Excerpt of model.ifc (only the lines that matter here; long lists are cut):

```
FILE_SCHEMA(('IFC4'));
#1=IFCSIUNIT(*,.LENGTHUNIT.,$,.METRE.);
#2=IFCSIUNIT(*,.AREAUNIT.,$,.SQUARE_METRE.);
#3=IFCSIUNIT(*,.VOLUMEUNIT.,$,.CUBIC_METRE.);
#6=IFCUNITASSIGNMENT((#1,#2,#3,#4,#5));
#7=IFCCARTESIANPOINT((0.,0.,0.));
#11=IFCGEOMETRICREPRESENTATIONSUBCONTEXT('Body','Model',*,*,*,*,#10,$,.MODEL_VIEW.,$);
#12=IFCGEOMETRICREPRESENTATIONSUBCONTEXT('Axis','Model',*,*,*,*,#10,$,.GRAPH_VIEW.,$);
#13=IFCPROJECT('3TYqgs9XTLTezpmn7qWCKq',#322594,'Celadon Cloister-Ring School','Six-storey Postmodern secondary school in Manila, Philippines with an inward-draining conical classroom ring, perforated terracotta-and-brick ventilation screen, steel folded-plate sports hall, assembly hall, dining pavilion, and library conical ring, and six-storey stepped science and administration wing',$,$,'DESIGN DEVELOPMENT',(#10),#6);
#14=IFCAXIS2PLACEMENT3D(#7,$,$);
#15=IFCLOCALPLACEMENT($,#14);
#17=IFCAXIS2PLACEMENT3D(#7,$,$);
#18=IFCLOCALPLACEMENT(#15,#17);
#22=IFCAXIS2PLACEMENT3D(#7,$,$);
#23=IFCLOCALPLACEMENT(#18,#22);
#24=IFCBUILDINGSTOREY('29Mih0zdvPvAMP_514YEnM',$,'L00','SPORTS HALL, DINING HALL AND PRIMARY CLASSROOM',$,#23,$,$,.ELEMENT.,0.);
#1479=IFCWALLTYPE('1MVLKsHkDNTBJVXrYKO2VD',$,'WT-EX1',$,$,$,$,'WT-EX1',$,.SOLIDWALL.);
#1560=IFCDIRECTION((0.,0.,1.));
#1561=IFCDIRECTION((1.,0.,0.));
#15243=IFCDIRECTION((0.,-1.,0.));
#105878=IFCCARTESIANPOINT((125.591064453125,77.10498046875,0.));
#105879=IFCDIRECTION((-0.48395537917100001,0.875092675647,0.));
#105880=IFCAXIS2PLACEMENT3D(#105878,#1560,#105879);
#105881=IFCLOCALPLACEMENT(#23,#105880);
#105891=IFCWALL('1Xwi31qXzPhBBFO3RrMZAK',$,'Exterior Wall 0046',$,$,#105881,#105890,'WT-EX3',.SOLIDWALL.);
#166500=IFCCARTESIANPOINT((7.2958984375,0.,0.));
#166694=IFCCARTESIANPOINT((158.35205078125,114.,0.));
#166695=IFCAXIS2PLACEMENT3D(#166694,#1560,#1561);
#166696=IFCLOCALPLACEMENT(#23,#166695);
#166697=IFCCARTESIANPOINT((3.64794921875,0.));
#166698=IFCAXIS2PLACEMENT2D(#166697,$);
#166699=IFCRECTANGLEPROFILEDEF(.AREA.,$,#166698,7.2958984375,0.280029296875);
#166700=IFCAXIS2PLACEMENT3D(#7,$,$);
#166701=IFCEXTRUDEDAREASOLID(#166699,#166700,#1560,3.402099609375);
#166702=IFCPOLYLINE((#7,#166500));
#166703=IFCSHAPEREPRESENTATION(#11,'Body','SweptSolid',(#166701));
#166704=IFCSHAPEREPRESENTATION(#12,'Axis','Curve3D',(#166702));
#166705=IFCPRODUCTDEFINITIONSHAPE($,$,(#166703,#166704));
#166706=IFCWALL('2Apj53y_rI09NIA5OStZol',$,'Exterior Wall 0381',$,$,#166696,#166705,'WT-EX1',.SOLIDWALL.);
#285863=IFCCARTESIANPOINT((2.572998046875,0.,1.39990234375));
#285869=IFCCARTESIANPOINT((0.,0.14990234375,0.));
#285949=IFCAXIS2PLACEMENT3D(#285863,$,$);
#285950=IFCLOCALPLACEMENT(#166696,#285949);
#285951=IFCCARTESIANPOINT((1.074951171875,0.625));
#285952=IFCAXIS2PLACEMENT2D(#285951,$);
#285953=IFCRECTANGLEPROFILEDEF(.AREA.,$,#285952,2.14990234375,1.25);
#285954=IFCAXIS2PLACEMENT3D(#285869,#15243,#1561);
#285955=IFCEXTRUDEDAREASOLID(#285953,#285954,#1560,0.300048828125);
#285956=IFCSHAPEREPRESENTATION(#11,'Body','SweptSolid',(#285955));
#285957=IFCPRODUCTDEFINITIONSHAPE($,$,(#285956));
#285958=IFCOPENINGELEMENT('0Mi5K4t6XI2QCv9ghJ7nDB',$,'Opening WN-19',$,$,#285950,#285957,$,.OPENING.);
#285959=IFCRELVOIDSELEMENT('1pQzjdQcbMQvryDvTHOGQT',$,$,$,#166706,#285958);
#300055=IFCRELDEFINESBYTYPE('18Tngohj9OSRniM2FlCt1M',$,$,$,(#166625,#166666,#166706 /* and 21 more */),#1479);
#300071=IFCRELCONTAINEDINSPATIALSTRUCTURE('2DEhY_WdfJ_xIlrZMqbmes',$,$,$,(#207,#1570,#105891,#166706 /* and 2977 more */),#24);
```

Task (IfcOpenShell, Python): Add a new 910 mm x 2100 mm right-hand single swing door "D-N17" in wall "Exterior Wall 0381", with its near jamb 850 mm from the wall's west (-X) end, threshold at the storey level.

```python
import numpy as np
import ifcopenshell
import ifcopenshell.api.feature
import ifcopenshell.api.geometry
import ifcopenshell.api.root
import ifcopenshell.api.spatial
import ifcopenshell.geom
import ifcopenshell.util.element
import ifcopenshell.util.placement
import ifcopenshell.util.representation
import ifcopenshell.util.shape
import ifcopenshell.util.unit

model = ifcopenshell.open("model.ifc")
unit_scale = ifcopenshell.util.unit.calculate_unit_scale(model)
settings = ifcopenshell.geom.settings()


def volume(element):
    """Net volume in cubic metres, openings subtracted."""
    shape = ifcopenshell.geom.create_shape(settings, element)
    return ifcopenshell.util.shape.get_volume(shape.geometry)


wall = model.by_id(166706)
storey = ifcopenshell.util.element.get_container(wall, ifc_class="IfcBuildingStorey")
context = ifcopenshell.util.representation.get_context(model, "Model", "Body", "MODEL_VIEW")
before = volume(wall)

width, height, from_end, sill = 0.91, 2.1, 0.85, 0.0  # metres

# The wall runs along its own X axis, and the end named is its -X end.
wall_shape = ifcopenshell.geom.create_shape(settings, wall)
x, y, z = ifcopenshell.util.shape.get_vertices(wall_shape.geometry).T
start = x.min() + from_end
face, thickness = float(y.min()), float(y.max() - y.min())
wall_matrix = ifcopenshell.util.placement.get_local_placement(wall.ObjectPlacement)
level = ifcopenshell.util.placement.get_local_placement(storey.ObjectPlacement)[2, 3]


def in_wall(x, y):
    """Placement at x, y metres in the wall's axes, at sill height."""
    matrix = wall_matrix.copy()
    matrix[:, 3] = wall_matrix @ np.array([x / unit_scale, y / unit_scale, 0.0, 1.0])
    matrix[2, 3] = level + sill / unit_scale
    return matrix


# Opening: a box that overshoots both wall faces by 50 mm.
opening = ifcopenshell.api.root.create_entity(model, ifc_class="IfcOpeningElement", predefined_type="OPENING")
box = ifcopenshell.api.geometry.add_wall_representation(
    model, context=context, length=width, height=height, thickness=thickness + 0.1
)
ifcopenshell.api.geometry.assign_representation(model, product=opening, representation=box)
ifcopenshell.api.geometry.edit_object_placement(model, product=opening, matrix=in_wall(start, face - 0.05), is_si=False)
ifcopenshell.api.feature.add_feature(model, feature=opening, element=wall)

door = ifcopenshell.api.root.create_entity(model, ifc_class="IfcDoor", name="D-N17", predefined_type="DOOR")
door.OverallWidth, door.OverallHeight = width / unit_scale, height / unit_scale
door.OperationType = "SINGLE_SWING_RIGHT"
body = ifcopenshell.api.geometry.add_door_representation(
    model,
    context=context,
    overall_width=door.OverallWidth,
    overall_height=door.OverallHeight,
    operation_type="SINGLE_SWING_RIGHT",
    lining_properties={"LiningDepth": thickness / unit_scale, "ThresholdDepth": thickness / unit_scale},
)
ifcopenshell.api.geometry.assign_representation(model, product=door, representation=body)
ifcopenshell.api.spatial.assign_container(model, products=[door], relating_structure=storey)
ifcopenshell.api.feature.add_filling(model, opening=opening, element=door)

# The lining spans the wall, so the door starts at the wall face.
ifcopenshell.api.geometry.edit_object_placement(model, product=door, matrix=in_wall(start, face), is_si=False)

after = volume(wall)

print(f"wall volume {before:.3f} -> {after:.3f} m3")

model.write("model_updated.ifc")
```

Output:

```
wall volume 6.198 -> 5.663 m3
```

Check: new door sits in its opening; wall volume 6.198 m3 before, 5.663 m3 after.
